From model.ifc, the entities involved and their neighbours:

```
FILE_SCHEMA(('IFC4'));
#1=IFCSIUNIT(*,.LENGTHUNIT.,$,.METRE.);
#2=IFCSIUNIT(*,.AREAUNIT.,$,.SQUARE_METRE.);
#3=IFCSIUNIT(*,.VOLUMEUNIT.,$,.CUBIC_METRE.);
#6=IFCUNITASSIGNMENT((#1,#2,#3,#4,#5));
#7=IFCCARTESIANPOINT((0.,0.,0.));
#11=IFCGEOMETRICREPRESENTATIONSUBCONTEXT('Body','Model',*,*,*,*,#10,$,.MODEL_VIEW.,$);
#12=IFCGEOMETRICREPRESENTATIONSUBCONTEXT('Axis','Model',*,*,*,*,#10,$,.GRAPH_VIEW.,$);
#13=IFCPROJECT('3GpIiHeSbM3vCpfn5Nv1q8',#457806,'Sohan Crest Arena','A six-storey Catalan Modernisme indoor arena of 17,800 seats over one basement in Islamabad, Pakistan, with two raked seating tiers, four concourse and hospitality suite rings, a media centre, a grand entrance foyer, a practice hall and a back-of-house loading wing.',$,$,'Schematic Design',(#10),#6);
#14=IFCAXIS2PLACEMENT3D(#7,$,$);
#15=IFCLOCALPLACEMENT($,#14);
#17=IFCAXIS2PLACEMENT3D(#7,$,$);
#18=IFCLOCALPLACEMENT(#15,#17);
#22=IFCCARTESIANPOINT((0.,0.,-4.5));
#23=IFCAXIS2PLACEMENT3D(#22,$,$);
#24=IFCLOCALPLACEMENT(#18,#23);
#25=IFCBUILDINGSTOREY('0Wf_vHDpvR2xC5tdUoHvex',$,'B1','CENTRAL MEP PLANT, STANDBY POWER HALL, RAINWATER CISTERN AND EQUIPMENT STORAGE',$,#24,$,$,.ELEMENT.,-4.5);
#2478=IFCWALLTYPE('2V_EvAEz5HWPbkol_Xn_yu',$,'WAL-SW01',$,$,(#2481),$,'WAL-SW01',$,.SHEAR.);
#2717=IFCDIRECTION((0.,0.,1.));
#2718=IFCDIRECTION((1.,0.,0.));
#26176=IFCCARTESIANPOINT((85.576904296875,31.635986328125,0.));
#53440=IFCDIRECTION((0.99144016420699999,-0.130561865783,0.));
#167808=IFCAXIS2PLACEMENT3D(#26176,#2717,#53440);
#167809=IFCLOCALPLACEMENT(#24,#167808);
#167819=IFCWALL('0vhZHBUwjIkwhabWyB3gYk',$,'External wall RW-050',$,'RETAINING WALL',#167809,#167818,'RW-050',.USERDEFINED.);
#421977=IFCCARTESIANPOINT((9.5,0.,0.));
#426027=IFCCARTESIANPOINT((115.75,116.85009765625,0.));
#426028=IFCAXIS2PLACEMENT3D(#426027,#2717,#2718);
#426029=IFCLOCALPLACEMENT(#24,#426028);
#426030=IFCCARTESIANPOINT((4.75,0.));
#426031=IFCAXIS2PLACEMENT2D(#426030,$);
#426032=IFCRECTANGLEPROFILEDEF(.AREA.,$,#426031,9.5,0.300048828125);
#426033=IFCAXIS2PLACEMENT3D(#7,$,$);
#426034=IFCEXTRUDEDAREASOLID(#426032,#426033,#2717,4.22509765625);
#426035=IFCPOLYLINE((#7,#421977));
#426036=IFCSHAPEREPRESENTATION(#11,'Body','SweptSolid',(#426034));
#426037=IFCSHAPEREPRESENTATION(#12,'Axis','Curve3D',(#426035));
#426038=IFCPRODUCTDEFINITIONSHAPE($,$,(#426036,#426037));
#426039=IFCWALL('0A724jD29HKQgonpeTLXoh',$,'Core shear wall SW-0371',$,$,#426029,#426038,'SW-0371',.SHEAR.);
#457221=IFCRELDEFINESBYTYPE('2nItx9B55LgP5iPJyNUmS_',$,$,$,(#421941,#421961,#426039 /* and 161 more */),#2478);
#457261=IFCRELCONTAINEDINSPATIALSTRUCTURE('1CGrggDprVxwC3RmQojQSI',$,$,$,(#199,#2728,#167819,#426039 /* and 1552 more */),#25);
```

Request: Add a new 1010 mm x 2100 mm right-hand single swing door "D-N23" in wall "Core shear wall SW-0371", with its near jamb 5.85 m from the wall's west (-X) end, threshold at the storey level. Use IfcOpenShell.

```python
import numpy as np
import ifcopenshell
import ifcopenshell.api.feature
import ifcopenshell.api.geometry
import ifcopenshell.api.root
import ifcopenshell.api.spatial
import ifcopenshell.geom
import ifcopenshell.util.element
import ifcopenshell.util.placement
import ifcopenshell.util.representation
import ifcopenshell.util.shape
import ifcopenshell.util.unit

model = ifcopenshell.open("model.ifc")
unit_scale = ifcopenshell.util.unit.calculate_unit_scale(model)
settings = ifcopenshell.geom.settings()


def volume(element):
    """Net volume in cubic metres, openings subtracted."""
    shape = ifcopenshell.geom.create_shape(settings, element)
    return ifcopenshell.util.shape.get_volume(shape.geometry)


wall = model.by_guid("0A724jD29HKQgonpeTLXoh")
storey = ifcopenshell.util.element.get_container(wall, ifc_class="IfcBuildingStorey")
context = ifcopenshell.util.representation.get_context(model, "Model", "Body", "MODEL_VIEW")
before = volume(wall)

width, height, from_end, sill = 1.01, 2.1, 5.85, 0.0  # metres

# The wall runs along its own X axis, and the end named is its -X end.
wall_shape = ifcopenshell.geom.create_shape(settings, wall)
x, y, z = ifcopenshell.util.shape.get_vertices(wall_shape.geometry).T
start = x.min() + from_end
face, thickness = float(y.min()), float(y.max() - y.min())
wall_matrix = ifcopenshell.util.placement.get_local_placement(wall.ObjectPlacement)
level = ifcopenshell.util.placement.get_local_placement(storey.ObjectPlacement)[2, 3]


def in_wall(x, y):
    """Placement at x, y metres in the wall's axes, at sill height."""
    matrix = wall_matrix.copy()
    matrix[:, 3] = wall_matrix @ np.array([x / unit_scale, y / unit_scale, 0.0, 1.0])
    matrix[2, 3] = level + sill / unit_scale
    return matrix


# Opening: a box that overshoots both wall faces by 50 mm.
opening = ifcopenshell.api.root.create_entity(model, ifc_class="IfcOpeningElement", predefined_type="OPENING")
box = ifcopenshell.api.geometry.add_wall_representation(
    model, context=context, length=width, height=height, thickness=thickness + 0.1
)
ifcopenshell.api.geometry.assign_representation(model, product=opening, representation=box)
ifcopenshell.api.geometry.edit_object_placement(model, product=opening, matrix=in_wall(start, face - 0.05), is_si=False)
ifcopenshell.api.feature.add_feature(model, feature=opening, element=wall)

door = ifcopenshell.api.root.create_entity(model, ifc_class="IfcDoor", name="D-N23", predefined_type="DOOR")
door.OverallWidth, door.OverallHeight = width / unit_scale, height / unit_scale
door.OperationType = "SINGLE_SWING_RIGHT"
body = ifcopenshell.api.geometry.add_door_representation(
    model,
    context=context,
    overall_width=door.OverallWidth,
    overall_height=door.OverallHeight,
    operation_type="SINGLE_SWING_RIGHT",
    lining_properties={"LiningDepth": thickness / unit_scale, "ThresholdDepth": thickness / unit_scale},
)
ifcopenshell.api.geometry.assign_representation(model, product=door, representation=body)
ifcopenshell.api.spatial.assign_container(model, products=[door], relating_structure=storey)
ifcopenshell.api.feature.add_filling(model, opening=opening, element=door)

# The lining spans the wall, so the door starts at the wall face.
ifcopenshell.api.geometry.edit_object_placement(model, product=door, matrix=in_wall(start, face), is_si=False)

after = volume(wall)

print(f"wall volume {before:.3f} -> {after:.3f} m3")

model.write("model_v2.ifc")
```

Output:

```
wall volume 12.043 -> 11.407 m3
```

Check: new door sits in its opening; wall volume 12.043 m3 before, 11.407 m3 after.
